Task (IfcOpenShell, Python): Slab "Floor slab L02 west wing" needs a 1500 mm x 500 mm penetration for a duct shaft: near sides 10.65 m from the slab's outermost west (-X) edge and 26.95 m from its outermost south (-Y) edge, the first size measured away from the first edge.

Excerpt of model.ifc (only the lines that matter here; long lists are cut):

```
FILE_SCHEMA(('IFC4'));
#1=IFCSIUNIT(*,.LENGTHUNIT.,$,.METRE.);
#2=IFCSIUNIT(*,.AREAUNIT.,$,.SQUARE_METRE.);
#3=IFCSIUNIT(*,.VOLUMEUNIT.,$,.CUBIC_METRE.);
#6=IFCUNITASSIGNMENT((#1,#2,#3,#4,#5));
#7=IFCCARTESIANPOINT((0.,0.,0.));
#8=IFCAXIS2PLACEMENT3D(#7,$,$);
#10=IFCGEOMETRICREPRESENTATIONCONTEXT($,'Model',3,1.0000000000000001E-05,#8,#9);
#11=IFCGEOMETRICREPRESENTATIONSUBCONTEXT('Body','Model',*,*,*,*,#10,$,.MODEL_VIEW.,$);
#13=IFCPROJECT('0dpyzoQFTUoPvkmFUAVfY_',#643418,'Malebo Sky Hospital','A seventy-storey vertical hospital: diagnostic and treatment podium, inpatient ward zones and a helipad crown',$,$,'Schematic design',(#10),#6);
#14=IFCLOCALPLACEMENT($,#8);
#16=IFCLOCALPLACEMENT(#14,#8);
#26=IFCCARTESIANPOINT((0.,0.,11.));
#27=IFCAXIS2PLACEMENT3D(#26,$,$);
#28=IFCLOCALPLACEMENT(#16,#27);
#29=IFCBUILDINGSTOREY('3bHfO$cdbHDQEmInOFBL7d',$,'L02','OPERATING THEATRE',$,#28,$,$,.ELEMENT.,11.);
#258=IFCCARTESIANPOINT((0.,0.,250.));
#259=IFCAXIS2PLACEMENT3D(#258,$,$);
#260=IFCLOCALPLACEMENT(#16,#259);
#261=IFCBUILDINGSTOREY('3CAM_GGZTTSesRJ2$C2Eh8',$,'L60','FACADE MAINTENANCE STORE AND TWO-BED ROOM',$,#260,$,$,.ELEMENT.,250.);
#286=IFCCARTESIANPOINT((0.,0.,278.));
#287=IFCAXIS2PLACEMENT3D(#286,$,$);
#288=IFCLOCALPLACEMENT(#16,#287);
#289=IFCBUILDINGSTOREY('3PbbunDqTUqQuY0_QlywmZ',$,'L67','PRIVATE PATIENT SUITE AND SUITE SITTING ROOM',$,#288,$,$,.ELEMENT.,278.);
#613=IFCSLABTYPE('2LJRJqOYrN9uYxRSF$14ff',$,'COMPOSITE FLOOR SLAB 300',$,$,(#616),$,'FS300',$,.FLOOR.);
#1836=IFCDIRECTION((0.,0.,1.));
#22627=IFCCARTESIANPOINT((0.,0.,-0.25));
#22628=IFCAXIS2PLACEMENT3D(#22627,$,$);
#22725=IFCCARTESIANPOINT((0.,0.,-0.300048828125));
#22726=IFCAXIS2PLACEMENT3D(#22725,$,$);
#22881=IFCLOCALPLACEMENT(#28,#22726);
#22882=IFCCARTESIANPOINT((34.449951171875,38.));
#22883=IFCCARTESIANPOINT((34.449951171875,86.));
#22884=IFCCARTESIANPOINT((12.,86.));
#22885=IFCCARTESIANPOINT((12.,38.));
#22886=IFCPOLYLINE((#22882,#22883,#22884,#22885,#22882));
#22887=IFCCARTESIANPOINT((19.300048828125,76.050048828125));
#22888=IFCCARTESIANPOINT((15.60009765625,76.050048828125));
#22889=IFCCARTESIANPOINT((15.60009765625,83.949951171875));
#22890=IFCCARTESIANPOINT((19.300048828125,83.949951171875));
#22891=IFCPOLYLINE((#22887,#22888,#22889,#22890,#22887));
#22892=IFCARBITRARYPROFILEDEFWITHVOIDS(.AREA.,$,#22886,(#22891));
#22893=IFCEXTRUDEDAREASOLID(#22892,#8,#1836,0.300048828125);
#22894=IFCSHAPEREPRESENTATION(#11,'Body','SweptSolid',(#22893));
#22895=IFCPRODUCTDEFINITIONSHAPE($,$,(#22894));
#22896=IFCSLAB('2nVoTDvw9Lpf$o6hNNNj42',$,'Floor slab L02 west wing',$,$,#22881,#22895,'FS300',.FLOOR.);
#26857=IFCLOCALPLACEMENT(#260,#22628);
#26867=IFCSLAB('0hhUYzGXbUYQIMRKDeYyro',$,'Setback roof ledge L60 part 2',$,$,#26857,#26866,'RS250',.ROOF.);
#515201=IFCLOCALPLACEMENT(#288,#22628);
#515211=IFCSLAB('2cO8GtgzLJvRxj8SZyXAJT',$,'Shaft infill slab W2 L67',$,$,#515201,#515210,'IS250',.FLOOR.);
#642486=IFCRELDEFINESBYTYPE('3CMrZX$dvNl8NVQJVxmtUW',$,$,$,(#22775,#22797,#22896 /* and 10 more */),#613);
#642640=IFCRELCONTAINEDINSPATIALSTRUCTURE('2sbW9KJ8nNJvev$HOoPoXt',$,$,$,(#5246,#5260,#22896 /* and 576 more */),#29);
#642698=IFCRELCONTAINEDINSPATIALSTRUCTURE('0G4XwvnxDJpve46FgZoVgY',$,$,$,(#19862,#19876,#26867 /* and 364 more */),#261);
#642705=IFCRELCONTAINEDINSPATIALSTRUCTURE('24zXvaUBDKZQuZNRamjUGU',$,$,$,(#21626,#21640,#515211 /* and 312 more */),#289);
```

```python
import numpy as np
import ifcopenshell
import ifcopenshell.api.feature
import ifcopenshell.api.geometry
import ifcopenshell.api.root
import ifcopenshell.geom
import ifcopenshell.util.placement
import ifcopenshell.util.representation
import ifcopenshell.util.shape
import ifcopenshell.util.unit

model = ifcopenshell.open("model.ifc")
unit_scale = ifcopenshell.util.unit.calculate_unit_scale(model)
settings = ifcopenshell.geom.settings()


def volume(element):
    """Net volume in cubic metres, openings subtracted."""
    shape = ifcopenshell.geom.create_shape(settings, element)
    return ifcopenshell.util.shape.get_volume(shape.geometry)


slab = model.by_id(22896)
before = volume(slab)

# Extent in the slab's own axes, in metres. The edges named are its -X and -Y sides.
slab_shape = ifcopenshell.geom.create_shape(settings, slab)
vertices = ifcopenshell.util.shape.get_vertices(slab_shape.geometry)
x_min, y_min, bottom = vertices.min(axis=0)
top = vertices[:, 2].max()

opening = ifcopenshell.api.root.create_entity(model, ifc_class="IfcOpeningElement", name="Duct shaft opening", predefined_type="OPENING")
context = ifcopenshell.util.representation.get_context(model, "Model", "Body", "MODEL_VIEW")
width, depth = 1.5, 0.5
outline = [(0.0, 0.0), (width, 0.0), (width, depth), (0.0, depth), (0.0, 0.0)]
# Overshoot both faces by 50 mm so the cut is clean.
shape = ifcopenshell.api.geometry.add_slab_representation(
    model, context=context, depth=top - bottom + 0.1, polyline=outline
)
ifcopenshell.api.geometry.assign_representation(model, product=opening, representation=shape)

matrix = ifcopenshell.util.placement.get_local_placement(slab.ObjectPlacement)
matrix[:, 3] = matrix @ np.append(np.array([x_min + 10.65, y_min + 26.95, bottom - 0.05]) / unit_scale, 1.0)
ifcopenshell.api.geometry.edit_object_placement(model, product=opening, matrix=matrix, is_si=False)
ifcopenshell.api.feature.add_feature(model, feature=opening, element=slab)

after = volume(slab)

print(f"slab volume {before:.3f} -> {after:.3f} m3")

model.write("model_rev.ifc")
```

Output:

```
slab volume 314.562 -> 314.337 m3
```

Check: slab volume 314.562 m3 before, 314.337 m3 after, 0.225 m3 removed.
